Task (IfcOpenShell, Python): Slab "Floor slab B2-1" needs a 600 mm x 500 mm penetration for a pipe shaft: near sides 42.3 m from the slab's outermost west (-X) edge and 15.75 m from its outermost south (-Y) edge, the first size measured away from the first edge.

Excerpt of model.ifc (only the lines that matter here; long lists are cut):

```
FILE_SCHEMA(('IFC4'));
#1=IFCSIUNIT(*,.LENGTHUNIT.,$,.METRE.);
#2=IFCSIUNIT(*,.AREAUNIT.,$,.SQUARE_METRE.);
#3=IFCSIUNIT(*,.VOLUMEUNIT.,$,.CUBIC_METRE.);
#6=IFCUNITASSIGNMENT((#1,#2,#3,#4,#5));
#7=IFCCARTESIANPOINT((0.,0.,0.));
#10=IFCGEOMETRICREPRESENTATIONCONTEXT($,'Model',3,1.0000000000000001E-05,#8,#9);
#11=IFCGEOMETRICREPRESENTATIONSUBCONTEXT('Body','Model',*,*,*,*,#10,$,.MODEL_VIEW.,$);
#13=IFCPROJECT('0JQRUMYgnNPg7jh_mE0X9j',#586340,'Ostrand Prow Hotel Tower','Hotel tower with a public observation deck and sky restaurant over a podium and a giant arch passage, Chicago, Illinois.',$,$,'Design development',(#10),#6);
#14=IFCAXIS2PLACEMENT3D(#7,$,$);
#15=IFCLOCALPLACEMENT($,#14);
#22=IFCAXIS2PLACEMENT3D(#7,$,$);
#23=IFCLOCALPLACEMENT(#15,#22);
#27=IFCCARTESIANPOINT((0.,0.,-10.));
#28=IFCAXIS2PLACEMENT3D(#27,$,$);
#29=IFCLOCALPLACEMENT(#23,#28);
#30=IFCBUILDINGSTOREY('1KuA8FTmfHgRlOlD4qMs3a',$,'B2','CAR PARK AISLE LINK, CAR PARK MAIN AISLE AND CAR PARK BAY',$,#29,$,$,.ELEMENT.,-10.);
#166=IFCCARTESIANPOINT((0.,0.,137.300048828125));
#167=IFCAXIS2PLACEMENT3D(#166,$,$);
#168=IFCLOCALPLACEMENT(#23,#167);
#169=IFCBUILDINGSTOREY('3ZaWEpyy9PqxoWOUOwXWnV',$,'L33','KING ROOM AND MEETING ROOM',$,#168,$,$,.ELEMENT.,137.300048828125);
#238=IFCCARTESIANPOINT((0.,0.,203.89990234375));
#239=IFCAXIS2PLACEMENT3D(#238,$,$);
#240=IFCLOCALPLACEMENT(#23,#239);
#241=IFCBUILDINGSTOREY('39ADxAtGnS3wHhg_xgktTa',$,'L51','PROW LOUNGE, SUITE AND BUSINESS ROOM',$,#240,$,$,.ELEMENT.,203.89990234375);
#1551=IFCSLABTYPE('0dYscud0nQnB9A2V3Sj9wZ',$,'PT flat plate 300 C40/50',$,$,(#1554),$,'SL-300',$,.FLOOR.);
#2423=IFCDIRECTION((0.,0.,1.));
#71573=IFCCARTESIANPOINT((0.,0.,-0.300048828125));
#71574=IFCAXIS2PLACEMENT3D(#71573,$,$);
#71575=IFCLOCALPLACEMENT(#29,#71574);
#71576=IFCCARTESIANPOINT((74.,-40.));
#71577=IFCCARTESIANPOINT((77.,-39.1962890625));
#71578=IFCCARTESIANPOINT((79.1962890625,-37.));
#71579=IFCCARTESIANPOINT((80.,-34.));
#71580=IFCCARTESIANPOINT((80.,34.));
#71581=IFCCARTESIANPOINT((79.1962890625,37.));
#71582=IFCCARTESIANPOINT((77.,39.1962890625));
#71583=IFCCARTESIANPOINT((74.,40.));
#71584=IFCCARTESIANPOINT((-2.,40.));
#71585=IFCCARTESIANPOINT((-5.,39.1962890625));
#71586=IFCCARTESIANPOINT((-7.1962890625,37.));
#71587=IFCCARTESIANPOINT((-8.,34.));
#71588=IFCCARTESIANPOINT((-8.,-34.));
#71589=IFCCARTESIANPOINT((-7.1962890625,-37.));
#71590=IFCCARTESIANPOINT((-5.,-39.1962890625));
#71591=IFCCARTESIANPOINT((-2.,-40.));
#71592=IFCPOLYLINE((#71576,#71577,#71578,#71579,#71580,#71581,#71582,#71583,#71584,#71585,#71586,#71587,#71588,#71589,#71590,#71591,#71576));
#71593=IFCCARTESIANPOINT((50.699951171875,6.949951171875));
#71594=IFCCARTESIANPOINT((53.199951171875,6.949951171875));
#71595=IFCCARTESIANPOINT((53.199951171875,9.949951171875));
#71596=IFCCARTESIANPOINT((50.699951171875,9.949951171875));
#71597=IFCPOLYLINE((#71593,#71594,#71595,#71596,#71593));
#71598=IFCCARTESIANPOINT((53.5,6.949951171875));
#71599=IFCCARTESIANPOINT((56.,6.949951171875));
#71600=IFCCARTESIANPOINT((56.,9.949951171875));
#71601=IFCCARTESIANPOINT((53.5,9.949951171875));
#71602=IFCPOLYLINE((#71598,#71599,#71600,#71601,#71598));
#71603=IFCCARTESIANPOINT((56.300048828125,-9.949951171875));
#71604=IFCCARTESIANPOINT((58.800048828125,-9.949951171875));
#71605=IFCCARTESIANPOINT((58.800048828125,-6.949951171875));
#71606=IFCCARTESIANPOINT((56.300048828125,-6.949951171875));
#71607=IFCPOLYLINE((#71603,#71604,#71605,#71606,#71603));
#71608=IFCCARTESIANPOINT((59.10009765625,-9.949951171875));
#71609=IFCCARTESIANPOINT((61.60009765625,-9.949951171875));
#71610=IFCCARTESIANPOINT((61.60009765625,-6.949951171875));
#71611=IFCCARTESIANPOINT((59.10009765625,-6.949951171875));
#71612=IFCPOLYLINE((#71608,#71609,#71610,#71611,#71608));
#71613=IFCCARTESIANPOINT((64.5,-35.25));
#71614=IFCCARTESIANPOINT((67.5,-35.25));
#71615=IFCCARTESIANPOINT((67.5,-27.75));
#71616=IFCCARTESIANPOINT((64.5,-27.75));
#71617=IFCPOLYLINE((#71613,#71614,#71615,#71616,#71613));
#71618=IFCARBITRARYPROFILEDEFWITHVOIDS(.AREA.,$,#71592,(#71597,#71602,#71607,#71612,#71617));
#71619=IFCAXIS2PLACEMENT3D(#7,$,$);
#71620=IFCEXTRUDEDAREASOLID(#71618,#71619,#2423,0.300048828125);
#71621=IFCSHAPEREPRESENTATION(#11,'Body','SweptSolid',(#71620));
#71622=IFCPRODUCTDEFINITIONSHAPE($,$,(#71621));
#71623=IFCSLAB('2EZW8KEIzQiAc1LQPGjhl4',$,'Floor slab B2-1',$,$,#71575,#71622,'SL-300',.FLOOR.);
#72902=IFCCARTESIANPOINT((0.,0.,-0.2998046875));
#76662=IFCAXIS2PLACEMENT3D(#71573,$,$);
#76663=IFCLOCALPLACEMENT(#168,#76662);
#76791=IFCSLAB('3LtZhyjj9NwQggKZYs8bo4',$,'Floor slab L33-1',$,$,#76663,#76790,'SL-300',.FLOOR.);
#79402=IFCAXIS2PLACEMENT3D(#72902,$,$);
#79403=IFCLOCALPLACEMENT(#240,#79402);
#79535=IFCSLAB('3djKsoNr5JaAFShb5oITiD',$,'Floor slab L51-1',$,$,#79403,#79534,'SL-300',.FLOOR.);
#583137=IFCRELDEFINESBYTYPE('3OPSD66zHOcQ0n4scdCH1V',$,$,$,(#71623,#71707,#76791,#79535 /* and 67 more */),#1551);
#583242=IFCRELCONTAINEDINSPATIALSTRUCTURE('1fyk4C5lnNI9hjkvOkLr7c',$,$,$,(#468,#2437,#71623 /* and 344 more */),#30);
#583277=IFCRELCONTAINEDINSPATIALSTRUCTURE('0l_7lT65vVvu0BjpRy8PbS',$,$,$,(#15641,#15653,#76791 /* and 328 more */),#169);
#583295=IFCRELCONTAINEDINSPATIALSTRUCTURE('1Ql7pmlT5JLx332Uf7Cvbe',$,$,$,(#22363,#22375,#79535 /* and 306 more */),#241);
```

```python
import numpy as np
import ifcopenshell
import ifcopenshell.api.feature
import ifcopenshell.api.geometry
import ifcopenshell.api.root
import ifcopenshell.geom
import ifcopenshell.util.placement
import ifcopenshell.util.representation
import ifcopenshell.util.shape
import ifcopenshell.util.unit

model = ifcopenshell.open("model.ifc")
unit_scale = ifcopenshell.util.unit.calculate_unit_scale(model)
settings = ifcopenshell.geom.settings()


def volume(element):
    """Net volume in cubic metres, openings subtracted."""
    shape = ifcopenshell.geom.create_shape(settings, element)
    return ifcopenshell.util.shape.get_volume(shape.geometry)


slab = model.by_guid("2EZW8KEIzQiAc1LQPGjhl4")
before = volume(slab)

# Extent in the slab's own axes, in metres. The edges named are its -X and -Y sides.
slab_shape = ifcopenshell.geom.create_shape(settings, slab)
vertices = ifcopenshell.util.shape.get_vertices(slab_shape.geometry)
x_min, y_min, bottom = vertices.min(axis=0)
top = vertices[:, 2].max()

opening = ifcopenshell.api.root.create_entity(model, ifc_class="IfcOpeningElement", name="Pipe shaft opening", predefined_type="OPENING")
context = ifcopenshell.util.representation.get_context(model, "Model", "Body", "MODEL_VIEW")
width, depth = 0.6, 0.5
outline = [(0.0, 0.0), (width, 0.0), (width, depth), (0.0, depth), (0.0, 0.0)]
# Overshoot both faces by 50 mm so the cut is clean.
shape = ifcopenshell.api.geometry.add_slab_representation(
    model, context=context, depth=top - bottom + 0.1, polyline=outline
)
ifcopenshell.api.geometry.assign_representation(model, product=opening, representation=shape)

matrix = ifcopenshell.util.placement.get_local_placement(slab.ObjectPlacement)
matrix[:, 3] = matrix @ np.append(np.array([x_min + 42.3, y_min + 15.75, bottom - 0.05]) / unit_scale, 1.0)
ifcopenshell.api.geometry.edit_object_placement(model, product=opening, matrix=matrix, is_si=False)
ifcopenshell.api.feature.add_feature(model, feature=opening, element=slab)

after = volume(slab)

print(f"slab volume {before:.3f} -> {after:.3f} m3")

model.write("model_rev.ifc")
```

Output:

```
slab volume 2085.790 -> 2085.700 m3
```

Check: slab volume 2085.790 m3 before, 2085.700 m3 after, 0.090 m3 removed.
